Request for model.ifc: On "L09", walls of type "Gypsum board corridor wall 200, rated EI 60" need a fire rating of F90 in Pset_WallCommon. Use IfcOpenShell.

First a look at what the model holds.

```python
import ifcopenshell
import ifcopenshell.util.element

model = ifcopenshell.open("model.ifc")
print(model.schema)
storey = next(s for s in model.by_type("IfcBuildingStorey") if s.Name == "L09")
walls = [e for e in ifcopenshell.util.element.get_decomposition(storey) if e.is_a("IfcWall")]
seen = {}
for e in walls:
    element_type = ifcopenshell.util.element.get_type(e)
    key = (element_type.Name if element_type != e and element_type else None, ifcopenshell.util.element.get_pset(e, "Pset_WallCommon", "FireRating"))
    seen[key] = seen.get(key, 0) + 1
for (name, value), count in sorted(seen.items(), key=str):
    print(count, "x", name, "|", value)
```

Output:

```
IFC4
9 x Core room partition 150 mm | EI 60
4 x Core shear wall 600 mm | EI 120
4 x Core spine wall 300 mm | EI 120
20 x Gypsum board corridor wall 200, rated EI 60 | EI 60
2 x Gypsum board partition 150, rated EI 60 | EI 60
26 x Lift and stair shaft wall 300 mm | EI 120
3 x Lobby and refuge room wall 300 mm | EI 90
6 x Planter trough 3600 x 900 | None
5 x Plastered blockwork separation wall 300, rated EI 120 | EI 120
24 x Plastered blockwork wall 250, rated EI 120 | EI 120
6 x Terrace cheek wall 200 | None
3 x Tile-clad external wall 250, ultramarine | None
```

```python
import ifcopenshell
import ifcopenshell.api.pset
import ifcopenshell.util.element

model = ifcopenshell.open("model.ifc")

storey = next(s for s in model.by_type("IfcBuildingStorey") if s.Name == "L09")
walls = [e for e in ifcopenshell.util.element.get_decomposition(storey) if e.is_a("IfcWall")]

count = 0
for e in walls:
    element_type = ifcopenshell.util.element.get_type(e)
    if element_type in (None, e) or element_type.Name != "Gypsum board corridor wall 200, rated EI 60":
        continue
    found = ifcopenshell.util.element.get_pset(e, "Pset_WallCommon", should_inherit=False)
    if found:
        pset = model.by_id(found["id"])
        if len(ifcopenshell.util.element.get_elements_by_pset(pset)) > 1:
            pset = ifcopenshell.api.pset.unshare_pset(model, products=[e], pset=pset)[0]
    else:
        pset = ifcopenshell.api.pset.add_pset(model, product=e, name="Pset_WallCommon")
    ifcopenshell.api.pset.edit_pset(model, pset=pset, properties={"FireRating": "F90"})
    count += 1

print(count, "walls updated")

model.write("model_updated.ifc")
```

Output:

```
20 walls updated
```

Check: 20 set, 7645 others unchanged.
